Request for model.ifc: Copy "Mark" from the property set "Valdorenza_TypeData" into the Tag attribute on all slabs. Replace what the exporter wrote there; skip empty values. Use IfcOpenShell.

First a look at what the model holds.

```python
import ifcopenshell
import ifcopenshell.util.element

model = ifcopenshell.open("model.ifc")
print(model.schema)
slabs = model.by_type("IfcSlab")
print(len(slabs), "slabs")
for e in slabs[:8]:
    source = ifcopenshell.util.element.get_pset(e, "Valdorenza_TypeData", "Mark")
    target = e.Tag
    print(e.id(), repr(source), repr(target), sep=" | ")
```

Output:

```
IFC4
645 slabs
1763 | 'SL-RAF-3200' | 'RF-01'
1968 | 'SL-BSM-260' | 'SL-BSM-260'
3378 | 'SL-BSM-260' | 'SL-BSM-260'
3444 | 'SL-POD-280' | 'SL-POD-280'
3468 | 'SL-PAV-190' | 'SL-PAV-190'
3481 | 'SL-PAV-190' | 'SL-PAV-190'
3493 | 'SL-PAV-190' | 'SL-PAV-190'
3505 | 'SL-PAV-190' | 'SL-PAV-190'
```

```python
import ifcopenshell
import ifcopenshell.util.element

model = ifcopenshell.open("model.ifc")

count = 0
for e in model.by_type("IfcSlab"):
    value = ifcopenshell.util.element.get_pset(e, "Valdorenza_TypeData", "Mark")
    current = e.Tag
    if not value or not value.strip() or current == value:
        continue
    e.Tag = value
    count += 1

print(count, "slabs updated")

model.write("model-out.ifc")
```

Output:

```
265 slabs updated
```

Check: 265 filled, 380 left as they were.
